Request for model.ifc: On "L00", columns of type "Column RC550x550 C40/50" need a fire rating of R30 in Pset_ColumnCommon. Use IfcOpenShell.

First a look at what the model holds.

```python
import ifcopenshell
import ifcopenshell.util.element

model = ifcopenshell.open("model.ifc")
print(model.schema)
storey = next(s for s in model.by_type("IfcBuildingStorey") if s.Name == "L00")
columns = [e for e in ifcopenshell.util.element.get_decomposition(storey) if e.is_a("IfcColumn")]
seen = {}
for e in columns:
    element_type = ifcopenshell.util.element.get_type(e)
    key = (element_type.Name if element_type != e and element_type else None, ifcopenshell.util.element.get_pset(e, "Pset_ColumnCommon", "FireRating"))
    seen[key] = seen.get(key, 0) + 1
for (name, value), count in sorted(seen.items(), key=str):
    print(count, "x", name, "|", value)
```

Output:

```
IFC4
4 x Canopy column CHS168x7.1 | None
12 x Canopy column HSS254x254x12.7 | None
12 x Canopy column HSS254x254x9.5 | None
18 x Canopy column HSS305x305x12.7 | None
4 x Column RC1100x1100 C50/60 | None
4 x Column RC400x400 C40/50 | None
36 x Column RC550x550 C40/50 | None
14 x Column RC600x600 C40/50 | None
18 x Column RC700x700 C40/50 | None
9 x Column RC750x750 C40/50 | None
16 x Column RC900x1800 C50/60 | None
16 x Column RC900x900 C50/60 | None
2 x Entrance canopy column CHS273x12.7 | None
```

```python
import ifcopenshell
import ifcopenshell.api.pset
import ifcopenshell.util.element

model = ifcopenshell.open("model.ifc")

storey = next(s for s in model.by_type("IfcBuildingStorey") if s.Name == "L00")
columns = [e for e in ifcopenshell.util.element.get_decomposition(storey) if e.is_a("IfcColumn")]

count = 0
for e in columns:
    element_type = ifcopenshell.util.element.get_type(e)
    if element_type in (None, e) or element_type.Name != "Column RC550x550 C40/50":
        continue
    # add_pset returns the element's existing set when there is one.
    pset = ifcopenshell.api.pset.add_pset(model, product=e, name="Pset_ColumnCommon")
    ifcopenshell.api.pset.edit_pset(model, pset=pset, properties={"FireRating": "R30"})
    count += 1

print(count, "columns updated")

model.write("model-out.ifc")
```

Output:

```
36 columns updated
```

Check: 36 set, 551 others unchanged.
